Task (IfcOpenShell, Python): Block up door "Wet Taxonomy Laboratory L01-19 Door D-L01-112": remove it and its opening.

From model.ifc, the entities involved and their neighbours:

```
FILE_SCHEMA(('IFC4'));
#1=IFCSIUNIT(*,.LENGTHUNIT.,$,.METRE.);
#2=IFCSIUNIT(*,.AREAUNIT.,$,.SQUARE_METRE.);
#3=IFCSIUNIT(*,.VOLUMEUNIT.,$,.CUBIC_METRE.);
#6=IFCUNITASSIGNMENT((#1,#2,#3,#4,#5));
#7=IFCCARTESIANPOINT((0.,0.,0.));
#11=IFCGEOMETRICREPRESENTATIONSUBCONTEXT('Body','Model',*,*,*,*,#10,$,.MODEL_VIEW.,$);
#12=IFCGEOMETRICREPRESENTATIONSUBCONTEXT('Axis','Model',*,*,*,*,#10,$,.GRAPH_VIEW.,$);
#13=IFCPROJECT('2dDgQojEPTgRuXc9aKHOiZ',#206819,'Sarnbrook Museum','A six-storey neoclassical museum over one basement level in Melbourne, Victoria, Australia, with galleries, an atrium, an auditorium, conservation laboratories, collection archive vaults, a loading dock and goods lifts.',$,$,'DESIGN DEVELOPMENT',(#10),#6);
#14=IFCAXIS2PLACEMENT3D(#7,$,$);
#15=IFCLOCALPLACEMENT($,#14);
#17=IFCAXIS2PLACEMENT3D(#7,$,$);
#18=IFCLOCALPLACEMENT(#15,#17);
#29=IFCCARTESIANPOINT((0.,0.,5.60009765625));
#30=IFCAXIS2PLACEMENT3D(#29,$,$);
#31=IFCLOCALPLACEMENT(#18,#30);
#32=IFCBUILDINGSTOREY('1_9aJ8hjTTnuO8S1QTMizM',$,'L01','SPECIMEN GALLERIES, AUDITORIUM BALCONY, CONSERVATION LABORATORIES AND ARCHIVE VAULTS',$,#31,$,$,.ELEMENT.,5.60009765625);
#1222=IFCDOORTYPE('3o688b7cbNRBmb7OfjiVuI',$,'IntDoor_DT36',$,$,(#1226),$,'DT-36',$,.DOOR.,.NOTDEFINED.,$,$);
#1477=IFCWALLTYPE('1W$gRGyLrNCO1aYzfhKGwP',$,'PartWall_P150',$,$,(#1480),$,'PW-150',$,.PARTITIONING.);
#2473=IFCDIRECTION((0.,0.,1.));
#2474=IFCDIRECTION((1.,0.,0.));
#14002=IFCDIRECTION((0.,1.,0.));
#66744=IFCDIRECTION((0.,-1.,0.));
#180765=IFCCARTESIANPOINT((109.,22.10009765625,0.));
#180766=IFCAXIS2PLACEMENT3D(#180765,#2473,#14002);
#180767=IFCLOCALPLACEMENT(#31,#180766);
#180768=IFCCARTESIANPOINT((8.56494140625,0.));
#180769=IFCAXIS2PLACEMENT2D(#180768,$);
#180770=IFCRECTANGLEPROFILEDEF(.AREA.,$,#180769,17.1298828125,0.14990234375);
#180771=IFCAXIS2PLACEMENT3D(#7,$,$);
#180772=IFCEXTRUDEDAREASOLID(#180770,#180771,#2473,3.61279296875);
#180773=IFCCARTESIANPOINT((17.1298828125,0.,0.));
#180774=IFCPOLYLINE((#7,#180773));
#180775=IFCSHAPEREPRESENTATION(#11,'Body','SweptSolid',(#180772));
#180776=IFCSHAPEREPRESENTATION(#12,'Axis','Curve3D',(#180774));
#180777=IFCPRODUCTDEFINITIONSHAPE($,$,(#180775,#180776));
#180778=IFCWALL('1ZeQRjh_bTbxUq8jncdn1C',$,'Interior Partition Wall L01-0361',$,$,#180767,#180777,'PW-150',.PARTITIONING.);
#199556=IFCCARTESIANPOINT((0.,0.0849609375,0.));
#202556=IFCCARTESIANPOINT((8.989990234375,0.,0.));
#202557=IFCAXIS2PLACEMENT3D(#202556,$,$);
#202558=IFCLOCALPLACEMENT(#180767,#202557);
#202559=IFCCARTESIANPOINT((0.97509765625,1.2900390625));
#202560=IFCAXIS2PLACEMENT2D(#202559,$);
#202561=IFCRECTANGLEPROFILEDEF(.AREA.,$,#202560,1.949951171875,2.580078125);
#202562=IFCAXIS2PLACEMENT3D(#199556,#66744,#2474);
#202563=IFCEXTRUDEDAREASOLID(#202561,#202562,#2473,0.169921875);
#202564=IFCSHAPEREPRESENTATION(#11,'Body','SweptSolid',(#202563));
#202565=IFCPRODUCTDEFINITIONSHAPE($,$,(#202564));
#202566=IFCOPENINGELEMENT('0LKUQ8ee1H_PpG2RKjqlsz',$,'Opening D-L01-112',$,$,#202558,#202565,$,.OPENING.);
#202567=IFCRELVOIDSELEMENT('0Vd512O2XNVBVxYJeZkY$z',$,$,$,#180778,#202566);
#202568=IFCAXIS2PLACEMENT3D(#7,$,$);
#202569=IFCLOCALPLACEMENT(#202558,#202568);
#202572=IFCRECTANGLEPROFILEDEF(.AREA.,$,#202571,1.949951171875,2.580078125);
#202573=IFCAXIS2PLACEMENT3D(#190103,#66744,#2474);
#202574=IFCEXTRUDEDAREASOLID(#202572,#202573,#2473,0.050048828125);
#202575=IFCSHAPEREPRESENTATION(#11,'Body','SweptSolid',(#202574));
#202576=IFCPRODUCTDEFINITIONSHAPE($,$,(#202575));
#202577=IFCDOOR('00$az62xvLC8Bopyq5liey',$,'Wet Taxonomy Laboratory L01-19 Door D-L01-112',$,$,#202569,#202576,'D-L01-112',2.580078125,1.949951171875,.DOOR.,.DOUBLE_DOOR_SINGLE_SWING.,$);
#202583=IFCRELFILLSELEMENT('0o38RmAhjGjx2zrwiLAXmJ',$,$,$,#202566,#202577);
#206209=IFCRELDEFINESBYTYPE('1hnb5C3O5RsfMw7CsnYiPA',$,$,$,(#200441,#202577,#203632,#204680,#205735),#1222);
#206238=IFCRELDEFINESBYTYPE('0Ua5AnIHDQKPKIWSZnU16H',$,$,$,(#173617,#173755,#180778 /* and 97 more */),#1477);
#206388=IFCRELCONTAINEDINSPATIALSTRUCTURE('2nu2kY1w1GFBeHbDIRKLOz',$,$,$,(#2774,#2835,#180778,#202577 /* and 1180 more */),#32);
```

```python
import ifcopenshell
import ifcopenshell.api.feature
import ifcopenshell.api.root
import ifcopenshell.geom
import ifcopenshell.util.shape

model = ifcopenshell.open("model.ifc")
settings = ifcopenshell.geom.settings()


def volume(element):
    """Net volume in cubic metres, openings subtracted."""
    shape = ifcopenshell.geom.create_shape(settings, element)
    return ifcopenshell.util.shape.get_volume(shape.geometry)


door = model.by_id(202577)
opening = door.FillsVoids[0].RelatingOpeningElement
wall = opening.VoidsElements[0].RelatingBuildingElement
before = volume(wall)

ifcopenshell.api.root.remove_product(model, product=door)
ifcopenshell.api.feature.remove_feature(model, feature=opening)

after = volume(wall)

print(f"wall volume {before:.3f} -> {after:.3f} m3")

model.write("model_updated.ifc")
```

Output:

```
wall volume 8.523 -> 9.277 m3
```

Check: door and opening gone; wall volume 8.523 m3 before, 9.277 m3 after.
